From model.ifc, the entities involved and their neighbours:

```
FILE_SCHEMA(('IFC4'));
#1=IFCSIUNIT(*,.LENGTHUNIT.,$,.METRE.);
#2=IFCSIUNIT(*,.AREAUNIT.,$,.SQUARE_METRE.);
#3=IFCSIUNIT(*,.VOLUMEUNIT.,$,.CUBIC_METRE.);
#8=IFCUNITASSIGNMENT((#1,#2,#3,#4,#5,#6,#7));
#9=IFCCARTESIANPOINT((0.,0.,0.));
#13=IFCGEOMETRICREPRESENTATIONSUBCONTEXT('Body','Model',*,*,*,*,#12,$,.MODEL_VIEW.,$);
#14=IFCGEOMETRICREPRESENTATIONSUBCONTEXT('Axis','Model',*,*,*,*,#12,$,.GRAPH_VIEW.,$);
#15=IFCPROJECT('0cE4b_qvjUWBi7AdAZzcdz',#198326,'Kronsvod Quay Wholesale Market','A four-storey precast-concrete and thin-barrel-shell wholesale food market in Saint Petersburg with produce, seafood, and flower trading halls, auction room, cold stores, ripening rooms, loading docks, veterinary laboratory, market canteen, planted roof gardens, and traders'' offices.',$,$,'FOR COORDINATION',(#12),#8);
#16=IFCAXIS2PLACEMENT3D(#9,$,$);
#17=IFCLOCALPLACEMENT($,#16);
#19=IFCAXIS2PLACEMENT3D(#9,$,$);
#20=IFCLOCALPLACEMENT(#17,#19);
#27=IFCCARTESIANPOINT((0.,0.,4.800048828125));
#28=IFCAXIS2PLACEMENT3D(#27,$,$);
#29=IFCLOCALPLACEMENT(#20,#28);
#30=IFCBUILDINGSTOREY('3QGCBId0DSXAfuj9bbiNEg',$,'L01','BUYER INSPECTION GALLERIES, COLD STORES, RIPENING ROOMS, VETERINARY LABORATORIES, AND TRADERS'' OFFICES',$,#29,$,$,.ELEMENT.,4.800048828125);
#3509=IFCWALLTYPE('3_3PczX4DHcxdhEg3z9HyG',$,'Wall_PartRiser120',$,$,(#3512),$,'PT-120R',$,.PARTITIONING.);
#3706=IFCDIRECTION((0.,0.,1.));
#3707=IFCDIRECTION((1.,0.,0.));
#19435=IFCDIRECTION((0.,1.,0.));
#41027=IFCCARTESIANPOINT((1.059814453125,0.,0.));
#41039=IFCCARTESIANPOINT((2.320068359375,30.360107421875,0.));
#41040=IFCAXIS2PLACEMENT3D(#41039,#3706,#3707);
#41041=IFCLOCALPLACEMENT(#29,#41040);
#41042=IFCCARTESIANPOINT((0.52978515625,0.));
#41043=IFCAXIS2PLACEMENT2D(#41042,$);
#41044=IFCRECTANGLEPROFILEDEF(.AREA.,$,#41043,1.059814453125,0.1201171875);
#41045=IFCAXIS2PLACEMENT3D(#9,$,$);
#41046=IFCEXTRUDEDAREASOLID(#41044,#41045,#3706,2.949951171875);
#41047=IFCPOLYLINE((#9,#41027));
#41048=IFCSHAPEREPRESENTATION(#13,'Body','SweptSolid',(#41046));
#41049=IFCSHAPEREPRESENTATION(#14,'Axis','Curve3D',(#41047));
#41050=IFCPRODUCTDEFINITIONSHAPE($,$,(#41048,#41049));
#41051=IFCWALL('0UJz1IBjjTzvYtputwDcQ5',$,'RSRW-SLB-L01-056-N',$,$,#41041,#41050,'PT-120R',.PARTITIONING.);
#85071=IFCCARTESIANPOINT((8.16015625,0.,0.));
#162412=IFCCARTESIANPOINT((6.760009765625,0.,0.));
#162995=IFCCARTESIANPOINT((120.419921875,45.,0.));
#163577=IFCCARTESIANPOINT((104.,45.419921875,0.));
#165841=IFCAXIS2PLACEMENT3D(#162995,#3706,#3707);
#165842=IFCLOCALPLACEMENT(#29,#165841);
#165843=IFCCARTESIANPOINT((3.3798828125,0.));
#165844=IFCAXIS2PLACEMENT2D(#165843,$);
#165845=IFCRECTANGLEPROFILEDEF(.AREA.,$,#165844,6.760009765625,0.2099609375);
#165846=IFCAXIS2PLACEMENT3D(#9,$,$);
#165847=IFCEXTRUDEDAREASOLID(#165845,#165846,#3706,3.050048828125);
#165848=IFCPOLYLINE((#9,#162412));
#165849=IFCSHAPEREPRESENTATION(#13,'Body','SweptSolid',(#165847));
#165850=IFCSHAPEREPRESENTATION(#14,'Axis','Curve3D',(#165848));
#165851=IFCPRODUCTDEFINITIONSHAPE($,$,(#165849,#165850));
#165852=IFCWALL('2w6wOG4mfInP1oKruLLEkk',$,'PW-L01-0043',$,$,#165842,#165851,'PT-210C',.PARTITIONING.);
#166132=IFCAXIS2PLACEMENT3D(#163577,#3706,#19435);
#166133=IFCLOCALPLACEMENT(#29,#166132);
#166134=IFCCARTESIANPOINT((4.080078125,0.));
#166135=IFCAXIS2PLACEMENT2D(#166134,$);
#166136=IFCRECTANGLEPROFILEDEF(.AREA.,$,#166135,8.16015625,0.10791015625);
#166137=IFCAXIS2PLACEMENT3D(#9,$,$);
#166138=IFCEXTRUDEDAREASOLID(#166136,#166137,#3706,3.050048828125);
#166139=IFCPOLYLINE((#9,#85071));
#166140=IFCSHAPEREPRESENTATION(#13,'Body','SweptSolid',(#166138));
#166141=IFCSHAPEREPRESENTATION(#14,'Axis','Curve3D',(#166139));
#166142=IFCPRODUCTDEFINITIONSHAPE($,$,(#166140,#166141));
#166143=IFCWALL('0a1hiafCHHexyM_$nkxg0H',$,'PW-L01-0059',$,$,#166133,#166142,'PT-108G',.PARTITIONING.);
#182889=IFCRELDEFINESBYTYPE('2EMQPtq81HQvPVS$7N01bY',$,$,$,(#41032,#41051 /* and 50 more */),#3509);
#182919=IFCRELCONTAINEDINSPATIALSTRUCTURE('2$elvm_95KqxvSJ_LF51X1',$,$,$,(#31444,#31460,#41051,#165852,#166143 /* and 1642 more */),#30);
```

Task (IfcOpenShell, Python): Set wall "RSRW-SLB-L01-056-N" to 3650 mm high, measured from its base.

```python
import ifcopenshell
import ifcopenshell.geom
import ifcopenshell.util.representation
import ifcopenshell.util.shape

model = ifcopenshell.open("model.ifc")
settings = ifcopenshell.geom.settings()


def volume(element):
    """Net volume in cubic metres, openings subtracted."""
    shape = ifcopenshell.geom.create_shape(settings, element)
    return ifcopenshell.util.shape.get_volume(shape.geometry)


wall = model.by_guid("0UJz1IBjjTzvYtputwDcQ5")
before = volume(wall)

body = ifcopenshell.util.representation.get_representation(wall, "Model", "Body")
solid = body.Items[0]
old_height = solid.Depth
solid.Depth = 3.65
after = volume(wall)

print(f"height {old_height:g} -> {solid.Depth:g}, volume {before:.3f} -> {after:.3f} m3")

model.write("model_v2.ifc")
```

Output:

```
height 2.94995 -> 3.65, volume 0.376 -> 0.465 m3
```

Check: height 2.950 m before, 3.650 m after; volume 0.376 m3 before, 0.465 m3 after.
